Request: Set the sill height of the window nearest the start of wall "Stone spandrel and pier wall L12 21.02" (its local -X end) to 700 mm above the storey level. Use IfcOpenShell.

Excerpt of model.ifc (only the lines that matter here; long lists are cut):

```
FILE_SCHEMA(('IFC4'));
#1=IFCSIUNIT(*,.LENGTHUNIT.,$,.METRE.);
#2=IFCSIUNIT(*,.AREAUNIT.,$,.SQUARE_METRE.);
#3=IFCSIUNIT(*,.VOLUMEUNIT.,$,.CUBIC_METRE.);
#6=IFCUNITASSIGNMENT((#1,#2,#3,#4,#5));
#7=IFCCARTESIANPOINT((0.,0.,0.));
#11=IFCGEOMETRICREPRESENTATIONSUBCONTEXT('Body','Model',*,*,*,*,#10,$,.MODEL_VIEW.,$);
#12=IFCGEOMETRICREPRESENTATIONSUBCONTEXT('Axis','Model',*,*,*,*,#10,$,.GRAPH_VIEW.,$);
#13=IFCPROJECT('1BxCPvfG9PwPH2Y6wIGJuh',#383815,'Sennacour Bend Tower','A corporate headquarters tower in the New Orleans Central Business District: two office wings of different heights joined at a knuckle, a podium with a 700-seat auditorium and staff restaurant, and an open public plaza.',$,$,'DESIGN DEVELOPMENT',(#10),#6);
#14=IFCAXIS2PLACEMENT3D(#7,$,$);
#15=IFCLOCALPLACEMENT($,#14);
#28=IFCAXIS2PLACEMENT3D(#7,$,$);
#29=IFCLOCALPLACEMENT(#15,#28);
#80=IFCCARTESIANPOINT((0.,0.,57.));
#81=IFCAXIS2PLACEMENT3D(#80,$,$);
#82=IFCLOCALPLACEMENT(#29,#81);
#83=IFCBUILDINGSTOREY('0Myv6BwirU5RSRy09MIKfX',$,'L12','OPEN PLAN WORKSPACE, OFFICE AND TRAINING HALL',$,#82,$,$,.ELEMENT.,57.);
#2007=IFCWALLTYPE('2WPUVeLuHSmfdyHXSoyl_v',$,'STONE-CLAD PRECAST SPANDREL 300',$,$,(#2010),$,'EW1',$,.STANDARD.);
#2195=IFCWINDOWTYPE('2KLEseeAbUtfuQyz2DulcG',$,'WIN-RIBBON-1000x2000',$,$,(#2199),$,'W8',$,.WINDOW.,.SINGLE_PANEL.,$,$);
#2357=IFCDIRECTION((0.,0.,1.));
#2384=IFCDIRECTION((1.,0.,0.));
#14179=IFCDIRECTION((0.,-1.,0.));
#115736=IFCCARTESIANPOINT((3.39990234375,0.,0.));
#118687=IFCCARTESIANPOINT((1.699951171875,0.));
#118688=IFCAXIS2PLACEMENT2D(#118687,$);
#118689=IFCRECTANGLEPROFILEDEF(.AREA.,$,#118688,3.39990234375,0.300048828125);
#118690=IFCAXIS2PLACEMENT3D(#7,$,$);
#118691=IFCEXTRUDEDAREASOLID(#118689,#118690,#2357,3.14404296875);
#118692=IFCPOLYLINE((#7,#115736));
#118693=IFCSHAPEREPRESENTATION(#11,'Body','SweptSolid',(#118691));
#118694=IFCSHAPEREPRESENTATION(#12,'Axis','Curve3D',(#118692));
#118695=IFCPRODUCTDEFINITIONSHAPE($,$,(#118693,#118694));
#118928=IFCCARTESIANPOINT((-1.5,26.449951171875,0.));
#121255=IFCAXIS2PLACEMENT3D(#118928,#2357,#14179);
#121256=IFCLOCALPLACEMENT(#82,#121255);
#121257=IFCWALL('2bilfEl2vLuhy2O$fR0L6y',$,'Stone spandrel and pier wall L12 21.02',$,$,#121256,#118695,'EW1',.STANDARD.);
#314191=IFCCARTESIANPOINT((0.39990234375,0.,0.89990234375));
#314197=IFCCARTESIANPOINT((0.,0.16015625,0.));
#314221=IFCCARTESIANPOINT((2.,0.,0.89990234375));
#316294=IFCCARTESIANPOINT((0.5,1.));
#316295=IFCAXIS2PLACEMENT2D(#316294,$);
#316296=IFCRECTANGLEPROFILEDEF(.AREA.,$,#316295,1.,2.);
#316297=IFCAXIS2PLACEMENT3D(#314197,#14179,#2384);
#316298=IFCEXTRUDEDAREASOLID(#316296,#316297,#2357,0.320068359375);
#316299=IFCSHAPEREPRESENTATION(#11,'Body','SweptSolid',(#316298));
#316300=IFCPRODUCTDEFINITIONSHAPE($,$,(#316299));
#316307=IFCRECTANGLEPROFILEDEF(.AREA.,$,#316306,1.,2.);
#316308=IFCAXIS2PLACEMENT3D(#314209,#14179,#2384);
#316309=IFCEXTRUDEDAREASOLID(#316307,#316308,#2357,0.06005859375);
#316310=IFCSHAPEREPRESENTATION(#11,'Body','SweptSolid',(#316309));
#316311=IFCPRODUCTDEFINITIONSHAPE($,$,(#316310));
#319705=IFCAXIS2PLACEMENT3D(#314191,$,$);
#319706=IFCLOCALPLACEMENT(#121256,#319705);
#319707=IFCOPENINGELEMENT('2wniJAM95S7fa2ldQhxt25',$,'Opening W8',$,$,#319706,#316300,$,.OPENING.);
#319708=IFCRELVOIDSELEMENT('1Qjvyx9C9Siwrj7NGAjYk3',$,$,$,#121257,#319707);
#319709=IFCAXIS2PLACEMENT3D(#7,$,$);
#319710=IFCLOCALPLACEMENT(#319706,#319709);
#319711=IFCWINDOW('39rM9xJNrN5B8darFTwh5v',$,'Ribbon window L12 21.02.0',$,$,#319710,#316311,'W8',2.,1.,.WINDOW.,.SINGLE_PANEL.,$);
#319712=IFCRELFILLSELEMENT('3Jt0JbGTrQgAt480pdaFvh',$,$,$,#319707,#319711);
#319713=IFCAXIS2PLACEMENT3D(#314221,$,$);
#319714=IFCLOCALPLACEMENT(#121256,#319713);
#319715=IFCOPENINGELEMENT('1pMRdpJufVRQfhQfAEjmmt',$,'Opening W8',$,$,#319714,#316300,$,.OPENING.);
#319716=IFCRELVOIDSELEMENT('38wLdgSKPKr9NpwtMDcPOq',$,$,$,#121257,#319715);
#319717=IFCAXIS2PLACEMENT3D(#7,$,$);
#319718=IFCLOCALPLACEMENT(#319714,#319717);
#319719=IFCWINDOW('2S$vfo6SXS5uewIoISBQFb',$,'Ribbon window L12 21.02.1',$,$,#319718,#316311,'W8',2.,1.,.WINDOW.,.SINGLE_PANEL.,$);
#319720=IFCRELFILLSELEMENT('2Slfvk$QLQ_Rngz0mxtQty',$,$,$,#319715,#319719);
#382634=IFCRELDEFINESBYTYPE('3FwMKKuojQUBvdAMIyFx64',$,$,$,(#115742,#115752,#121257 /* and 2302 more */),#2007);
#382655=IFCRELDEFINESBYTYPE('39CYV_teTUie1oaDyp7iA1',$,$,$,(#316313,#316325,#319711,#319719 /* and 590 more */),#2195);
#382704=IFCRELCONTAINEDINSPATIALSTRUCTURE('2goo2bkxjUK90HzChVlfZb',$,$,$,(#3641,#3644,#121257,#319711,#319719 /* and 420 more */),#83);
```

```python
import numpy as np
import ifcopenshell
import ifcopenshell.api.geometry
import ifcopenshell.geom
import ifcopenshell.util.element
import ifcopenshell.util.placement
import ifcopenshell.util.shape
import ifcopenshell.util.unit

model = ifcopenshell.open("model.ifc")
unit_scale = ifcopenshell.util.unit.calculate_unit_scale(model)

window = model.by_guid("39rM9xJNrN5B8darFTwh5v")
opening = window.FillsVoids[0].RelatingOpeningElement
storey = ifcopenshell.util.element.get_container(window, ifc_class="IfcBuildingStorey")
level = ifcopenshell.util.placement.get_local_placement(storey.ObjectPlacement)[2, 3]

# The opening's origin need not be at the sill, so measure its lowest point.
shape = ifcopenshell.geom.create_shape(ifcopenshell.geom.settings(), opening)
bottom = ifcopenshell.util.shape.get_shape_bottom_elevation(shape, shape.geometry) / unit_scale
dz = level + 0.7 / unit_scale - bottom

shift = np.array([0.0, 0.0, dz])
# The window is placed relative to its opening, so it follows when the opening moves.
matrix = ifcopenshell.util.placement.get_local_placement(opening.ObjectPlacement)
matrix[:3, 3] += shift
ifcopenshell.api.geometry.edit_object_placement(
    model, product=opening, matrix=matrix, is_si=False, should_transform_children=True
)

print(f"moved by {dz * unit_scale:+.3f} m")

model.write("model_rev.ifc")
```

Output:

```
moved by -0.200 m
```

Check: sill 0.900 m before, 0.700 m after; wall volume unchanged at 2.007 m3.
